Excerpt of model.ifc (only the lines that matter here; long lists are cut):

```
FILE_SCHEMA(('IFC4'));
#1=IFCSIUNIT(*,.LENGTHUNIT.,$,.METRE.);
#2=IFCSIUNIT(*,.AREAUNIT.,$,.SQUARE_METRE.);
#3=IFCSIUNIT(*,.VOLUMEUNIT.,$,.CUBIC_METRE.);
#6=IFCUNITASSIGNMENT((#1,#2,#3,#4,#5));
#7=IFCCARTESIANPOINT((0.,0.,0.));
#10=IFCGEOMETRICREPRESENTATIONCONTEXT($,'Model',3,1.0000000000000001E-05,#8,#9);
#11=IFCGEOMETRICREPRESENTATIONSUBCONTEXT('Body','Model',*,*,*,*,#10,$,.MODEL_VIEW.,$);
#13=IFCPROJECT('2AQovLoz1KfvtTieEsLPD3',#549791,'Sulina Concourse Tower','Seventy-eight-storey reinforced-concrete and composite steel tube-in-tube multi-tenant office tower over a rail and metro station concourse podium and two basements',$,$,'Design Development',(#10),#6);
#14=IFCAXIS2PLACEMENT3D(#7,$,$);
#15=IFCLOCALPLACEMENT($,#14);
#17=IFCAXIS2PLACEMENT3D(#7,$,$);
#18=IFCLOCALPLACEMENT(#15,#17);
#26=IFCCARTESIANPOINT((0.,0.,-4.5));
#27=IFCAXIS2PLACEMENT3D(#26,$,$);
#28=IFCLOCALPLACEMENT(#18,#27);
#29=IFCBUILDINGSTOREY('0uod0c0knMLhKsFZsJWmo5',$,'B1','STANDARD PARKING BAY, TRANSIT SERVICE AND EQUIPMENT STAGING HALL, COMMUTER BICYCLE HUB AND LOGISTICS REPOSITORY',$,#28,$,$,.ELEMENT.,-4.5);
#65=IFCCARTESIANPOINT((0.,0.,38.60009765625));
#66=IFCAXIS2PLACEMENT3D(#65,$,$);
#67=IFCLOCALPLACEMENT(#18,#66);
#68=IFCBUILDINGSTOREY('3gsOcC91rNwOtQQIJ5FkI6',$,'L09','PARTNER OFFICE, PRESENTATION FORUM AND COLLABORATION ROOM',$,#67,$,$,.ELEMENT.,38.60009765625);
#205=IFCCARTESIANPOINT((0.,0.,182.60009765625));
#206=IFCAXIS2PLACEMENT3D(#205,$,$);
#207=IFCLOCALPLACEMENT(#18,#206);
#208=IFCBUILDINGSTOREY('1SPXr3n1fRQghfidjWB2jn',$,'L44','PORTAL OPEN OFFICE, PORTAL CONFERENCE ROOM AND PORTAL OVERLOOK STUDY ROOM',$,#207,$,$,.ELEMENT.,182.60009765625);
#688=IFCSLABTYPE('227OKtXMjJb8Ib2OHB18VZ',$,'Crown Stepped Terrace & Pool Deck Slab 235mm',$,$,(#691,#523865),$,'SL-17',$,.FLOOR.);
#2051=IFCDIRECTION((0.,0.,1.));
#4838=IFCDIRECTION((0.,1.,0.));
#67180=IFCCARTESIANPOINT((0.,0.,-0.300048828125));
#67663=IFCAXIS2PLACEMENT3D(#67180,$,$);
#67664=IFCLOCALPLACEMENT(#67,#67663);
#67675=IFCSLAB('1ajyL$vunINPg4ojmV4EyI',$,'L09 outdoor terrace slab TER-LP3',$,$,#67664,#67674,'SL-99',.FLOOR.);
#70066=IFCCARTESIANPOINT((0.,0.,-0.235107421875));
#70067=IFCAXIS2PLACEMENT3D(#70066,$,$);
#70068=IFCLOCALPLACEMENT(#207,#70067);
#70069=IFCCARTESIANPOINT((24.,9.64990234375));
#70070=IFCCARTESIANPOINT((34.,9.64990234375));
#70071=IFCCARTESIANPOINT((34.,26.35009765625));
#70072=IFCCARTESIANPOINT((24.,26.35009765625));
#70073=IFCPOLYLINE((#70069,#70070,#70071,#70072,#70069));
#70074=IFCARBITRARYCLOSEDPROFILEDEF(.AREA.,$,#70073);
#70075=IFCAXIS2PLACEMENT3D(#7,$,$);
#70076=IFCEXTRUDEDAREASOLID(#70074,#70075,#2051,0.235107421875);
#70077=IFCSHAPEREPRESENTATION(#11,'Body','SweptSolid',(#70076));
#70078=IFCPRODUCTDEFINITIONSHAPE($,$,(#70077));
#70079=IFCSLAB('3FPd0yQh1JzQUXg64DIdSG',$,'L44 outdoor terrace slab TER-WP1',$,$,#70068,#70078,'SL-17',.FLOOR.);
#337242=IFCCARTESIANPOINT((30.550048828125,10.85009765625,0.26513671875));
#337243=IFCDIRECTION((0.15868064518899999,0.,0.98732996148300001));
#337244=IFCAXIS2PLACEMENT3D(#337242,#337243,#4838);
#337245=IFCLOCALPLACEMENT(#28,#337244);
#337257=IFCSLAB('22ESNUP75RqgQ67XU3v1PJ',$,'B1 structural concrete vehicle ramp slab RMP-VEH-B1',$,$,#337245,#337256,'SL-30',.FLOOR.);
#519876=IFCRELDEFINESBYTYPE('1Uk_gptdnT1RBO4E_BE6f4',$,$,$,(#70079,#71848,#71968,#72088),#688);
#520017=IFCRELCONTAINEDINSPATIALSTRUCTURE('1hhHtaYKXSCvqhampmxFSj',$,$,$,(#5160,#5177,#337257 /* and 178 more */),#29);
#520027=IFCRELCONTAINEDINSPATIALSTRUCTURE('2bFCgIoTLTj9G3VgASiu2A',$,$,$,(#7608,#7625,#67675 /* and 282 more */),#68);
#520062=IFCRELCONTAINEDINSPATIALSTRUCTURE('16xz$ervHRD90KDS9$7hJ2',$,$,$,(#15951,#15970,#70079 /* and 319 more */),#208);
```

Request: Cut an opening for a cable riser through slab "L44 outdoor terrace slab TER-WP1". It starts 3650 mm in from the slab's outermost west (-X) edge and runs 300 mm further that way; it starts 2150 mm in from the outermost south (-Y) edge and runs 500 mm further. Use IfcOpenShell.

```python
import numpy as np
import ifcopenshell
import ifcopenshell.api.feature
import ifcopenshell.api.geometry
import ifcopenshell.api.root
import ifcopenshell.geom
import ifcopenshell.util.placement
import ifcopenshell.util.representation
import ifcopenshell.util.shape
import ifcopenshell.util.unit

model = ifcopenshell.open("model.ifc")
unit_scale = ifcopenshell.util.unit.calculate_unit_scale(model)
settings = ifcopenshell.geom.settings()


def volume(element):
    """Net volume in cubic metres, openings subtracted."""
    shape = ifcopenshell.geom.create_shape(settings, element)
    return ifcopenshell.util.shape.get_volume(shape.geometry)


slab = model.by_guid("3FPd0yQh1JzQUXg64DIdSG")
before = volume(slab)

# Extent in the slab's own axes, in metres. The edges named are its -X and -Y sides.
slab_shape = ifcopenshell.geom.create_shape(settings, slab)
vertices = ifcopenshell.util.shape.get_vertices(slab_shape.geometry)
x_min, y_min, bottom = vertices.min(axis=0)
top = vertices[:, 2].max()

opening = ifcopenshell.api.root.create_entity(model, ifc_class="IfcOpeningElement", name="Cable riser opening", predefined_type="OPENING")
context = ifcopenshell.util.representation.get_context(model, "Model", "Body", "MODEL_VIEW")
width, depth = 0.3, 0.5
outline = [(0.0, 0.0), (width, 0.0), (width, depth), (0.0, depth), (0.0, 0.0)]
# Overshoot both faces by 50 mm so the cut is clean.
shape = ifcopenshell.api.geometry.add_slab_representation(
    model, context=context, depth=top - bottom + 0.1, polyline=outline
)
ifcopenshell.api.geometry.assign_representation(model, product=opening, representation=shape)

matrix = ifcopenshell.util.placement.get_local_placement(slab.ObjectPlacement)
matrix[:, 3] = matrix @ np.append(np.array([x_min + 3.65, y_min + 2.15, bottom - 0.05]) / unit_scale, 1.0)
ifcopenshell.api.geometry.edit_object_placement(model, product=opening, matrix=matrix, is_si=False)
ifcopenshell.api.feature.add_feature(model, feature=opening, element=slab)

after = volume(slab)

print(f"slab volume {before:.3f} -> {after:.3f} m3")

model.write("model_edited.ifc")
```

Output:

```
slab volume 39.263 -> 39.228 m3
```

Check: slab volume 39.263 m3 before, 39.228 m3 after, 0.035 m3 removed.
